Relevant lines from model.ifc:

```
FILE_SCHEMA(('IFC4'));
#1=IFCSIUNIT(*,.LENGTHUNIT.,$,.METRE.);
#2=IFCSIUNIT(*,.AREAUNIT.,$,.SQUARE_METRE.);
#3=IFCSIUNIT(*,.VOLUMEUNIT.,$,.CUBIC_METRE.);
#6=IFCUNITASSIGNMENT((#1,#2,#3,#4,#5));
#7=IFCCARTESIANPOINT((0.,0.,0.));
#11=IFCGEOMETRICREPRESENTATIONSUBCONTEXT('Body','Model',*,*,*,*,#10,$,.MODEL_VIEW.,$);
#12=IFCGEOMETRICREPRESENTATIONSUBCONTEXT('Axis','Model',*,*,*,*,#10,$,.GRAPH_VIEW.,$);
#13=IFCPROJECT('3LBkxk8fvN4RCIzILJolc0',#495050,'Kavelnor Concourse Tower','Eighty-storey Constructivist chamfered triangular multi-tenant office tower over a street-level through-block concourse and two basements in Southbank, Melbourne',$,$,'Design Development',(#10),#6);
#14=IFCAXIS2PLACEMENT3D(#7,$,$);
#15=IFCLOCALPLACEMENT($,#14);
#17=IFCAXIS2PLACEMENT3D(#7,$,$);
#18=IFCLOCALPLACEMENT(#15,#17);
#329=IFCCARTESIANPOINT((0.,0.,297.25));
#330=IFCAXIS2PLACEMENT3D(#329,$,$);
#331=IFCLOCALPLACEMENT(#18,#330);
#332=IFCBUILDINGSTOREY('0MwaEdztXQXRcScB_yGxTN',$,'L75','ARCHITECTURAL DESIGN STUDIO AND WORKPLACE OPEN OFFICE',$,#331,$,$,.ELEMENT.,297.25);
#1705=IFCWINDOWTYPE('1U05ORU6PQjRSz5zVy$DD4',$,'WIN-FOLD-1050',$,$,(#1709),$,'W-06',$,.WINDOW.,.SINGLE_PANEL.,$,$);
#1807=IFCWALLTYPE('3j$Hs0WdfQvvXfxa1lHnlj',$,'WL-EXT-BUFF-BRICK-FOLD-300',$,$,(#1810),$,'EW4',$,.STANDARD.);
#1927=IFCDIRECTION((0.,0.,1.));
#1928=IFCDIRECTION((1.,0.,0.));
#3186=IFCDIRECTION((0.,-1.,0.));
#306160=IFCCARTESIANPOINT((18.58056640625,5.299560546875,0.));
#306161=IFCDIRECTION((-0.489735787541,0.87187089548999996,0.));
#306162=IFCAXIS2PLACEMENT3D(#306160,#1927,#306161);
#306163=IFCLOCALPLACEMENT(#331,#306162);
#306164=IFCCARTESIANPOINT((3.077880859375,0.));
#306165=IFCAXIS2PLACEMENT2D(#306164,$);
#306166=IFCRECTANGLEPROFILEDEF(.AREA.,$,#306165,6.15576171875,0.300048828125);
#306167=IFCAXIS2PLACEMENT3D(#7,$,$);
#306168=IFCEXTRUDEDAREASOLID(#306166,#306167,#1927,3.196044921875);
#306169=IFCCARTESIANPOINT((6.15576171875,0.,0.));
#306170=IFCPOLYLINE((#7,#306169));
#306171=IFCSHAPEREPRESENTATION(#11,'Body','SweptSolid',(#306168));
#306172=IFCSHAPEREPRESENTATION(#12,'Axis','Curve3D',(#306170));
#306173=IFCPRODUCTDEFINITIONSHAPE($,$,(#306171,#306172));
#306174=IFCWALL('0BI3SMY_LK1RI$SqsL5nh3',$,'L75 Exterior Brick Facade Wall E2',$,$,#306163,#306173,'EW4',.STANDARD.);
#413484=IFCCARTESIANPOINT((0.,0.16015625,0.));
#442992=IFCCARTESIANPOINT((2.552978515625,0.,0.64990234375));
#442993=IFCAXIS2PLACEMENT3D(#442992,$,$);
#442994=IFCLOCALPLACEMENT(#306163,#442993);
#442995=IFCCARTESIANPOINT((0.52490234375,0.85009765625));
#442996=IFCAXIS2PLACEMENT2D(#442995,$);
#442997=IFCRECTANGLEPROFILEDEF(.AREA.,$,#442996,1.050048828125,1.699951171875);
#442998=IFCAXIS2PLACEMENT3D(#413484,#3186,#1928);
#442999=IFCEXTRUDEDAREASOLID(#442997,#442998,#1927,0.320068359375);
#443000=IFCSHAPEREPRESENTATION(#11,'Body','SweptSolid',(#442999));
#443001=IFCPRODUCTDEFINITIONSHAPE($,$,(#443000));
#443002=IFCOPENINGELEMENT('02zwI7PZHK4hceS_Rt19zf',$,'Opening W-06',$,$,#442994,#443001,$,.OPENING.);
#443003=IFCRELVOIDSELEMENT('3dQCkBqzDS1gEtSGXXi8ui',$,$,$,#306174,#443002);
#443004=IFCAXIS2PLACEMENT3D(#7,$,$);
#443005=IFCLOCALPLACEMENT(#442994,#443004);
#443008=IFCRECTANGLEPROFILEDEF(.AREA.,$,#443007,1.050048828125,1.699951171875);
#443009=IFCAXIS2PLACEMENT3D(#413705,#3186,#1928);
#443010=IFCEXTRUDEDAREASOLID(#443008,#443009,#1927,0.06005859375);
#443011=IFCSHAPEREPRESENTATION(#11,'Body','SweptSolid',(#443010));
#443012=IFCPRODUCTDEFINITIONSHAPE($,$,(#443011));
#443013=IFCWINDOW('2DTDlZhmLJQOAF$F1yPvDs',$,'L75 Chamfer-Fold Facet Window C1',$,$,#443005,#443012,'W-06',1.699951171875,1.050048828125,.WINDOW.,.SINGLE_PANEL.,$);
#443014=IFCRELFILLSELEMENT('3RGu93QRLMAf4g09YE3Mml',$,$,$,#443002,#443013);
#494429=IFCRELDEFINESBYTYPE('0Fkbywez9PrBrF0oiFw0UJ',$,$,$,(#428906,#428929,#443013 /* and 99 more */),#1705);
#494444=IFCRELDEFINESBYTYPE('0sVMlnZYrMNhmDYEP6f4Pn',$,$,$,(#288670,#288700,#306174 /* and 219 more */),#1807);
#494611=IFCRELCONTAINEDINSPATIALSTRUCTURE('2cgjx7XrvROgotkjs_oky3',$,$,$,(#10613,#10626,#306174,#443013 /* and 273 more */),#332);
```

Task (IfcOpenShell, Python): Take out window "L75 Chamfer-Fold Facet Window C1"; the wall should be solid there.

```python
import ifcopenshell
import ifcopenshell.api.feature
import ifcopenshell.api.root
import ifcopenshell.geom
import ifcopenshell.util.shape

model = ifcopenshell.open("model.ifc")
settings = ifcopenshell.geom.settings()


def volume(element):
    """Net volume in cubic metres, openings subtracted."""
    shape = ifcopenshell.geom.create_shape(settings, element)
    return ifcopenshell.util.shape.get_volume(shape.geometry)


window = model.by_id(443013)
opening = window.FillsVoids[0].RelatingOpeningElement
wall = opening.VoidsElements[0].RelatingBuildingElement
before = volume(wall)

ifcopenshell.api.root.remove_product(model, product=window)
ifcopenshell.api.feature.remove_feature(model, feature=opening)

after = volume(wall)

print(f"wall volume {before:.3f} -> {after:.3f} m3")

model.write("model_v2.ifc")
```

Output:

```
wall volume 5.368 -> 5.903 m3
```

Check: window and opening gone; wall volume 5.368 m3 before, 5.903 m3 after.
